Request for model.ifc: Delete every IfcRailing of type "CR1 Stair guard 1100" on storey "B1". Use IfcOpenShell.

First a look at what the model holds.

```python
import ifcopenshell
import ifcopenshell.util.element

model = ifcopenshell.open("model.ifc")
print(model.schema)
storey = next(s for s in model.by_type("IfcBuildingStorey") if s.Name == "B1")
railings = [e for e in ifcopenshell.util.element.get_decomposition(storey) if e.is_a("IfcRailing")]
seen = {}
for e in railings:
    element_type = ifcopenshell.util.element.get_type(e)
    name = element_type.Name if element_type not in (None, e) else None
    seen[name] = seen.get(name, 0) + 1
for name, count in sorted(seen.items(), key=str):
    print(count, "x", name)
```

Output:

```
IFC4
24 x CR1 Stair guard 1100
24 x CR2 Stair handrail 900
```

```python
import ifcopenshell
import ifcopenshell.api.root
import ifcopenshell.util.element

model = ifcopenshell.open("model.ifc")

storey = next(s for s in model.by_type("IfcBuildingStorey") if s.Name == "B1")
railings = [e for e in ifcopenshell.util.element.get_decomposition(storey) if e.is_a("IfcRailing")]
targets = [e for e in railings if (t := ifcopenshell.util.element.get_type(e)) not in (None, e) and t.Name == "CR1 Stair guard 1100"]

for e in targets:
    ifcopenshell.api.root.remove_product(model, product=e)
print(len(targets), "removed")

model.write("model_updated.ifc")
```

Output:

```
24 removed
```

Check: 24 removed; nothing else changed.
